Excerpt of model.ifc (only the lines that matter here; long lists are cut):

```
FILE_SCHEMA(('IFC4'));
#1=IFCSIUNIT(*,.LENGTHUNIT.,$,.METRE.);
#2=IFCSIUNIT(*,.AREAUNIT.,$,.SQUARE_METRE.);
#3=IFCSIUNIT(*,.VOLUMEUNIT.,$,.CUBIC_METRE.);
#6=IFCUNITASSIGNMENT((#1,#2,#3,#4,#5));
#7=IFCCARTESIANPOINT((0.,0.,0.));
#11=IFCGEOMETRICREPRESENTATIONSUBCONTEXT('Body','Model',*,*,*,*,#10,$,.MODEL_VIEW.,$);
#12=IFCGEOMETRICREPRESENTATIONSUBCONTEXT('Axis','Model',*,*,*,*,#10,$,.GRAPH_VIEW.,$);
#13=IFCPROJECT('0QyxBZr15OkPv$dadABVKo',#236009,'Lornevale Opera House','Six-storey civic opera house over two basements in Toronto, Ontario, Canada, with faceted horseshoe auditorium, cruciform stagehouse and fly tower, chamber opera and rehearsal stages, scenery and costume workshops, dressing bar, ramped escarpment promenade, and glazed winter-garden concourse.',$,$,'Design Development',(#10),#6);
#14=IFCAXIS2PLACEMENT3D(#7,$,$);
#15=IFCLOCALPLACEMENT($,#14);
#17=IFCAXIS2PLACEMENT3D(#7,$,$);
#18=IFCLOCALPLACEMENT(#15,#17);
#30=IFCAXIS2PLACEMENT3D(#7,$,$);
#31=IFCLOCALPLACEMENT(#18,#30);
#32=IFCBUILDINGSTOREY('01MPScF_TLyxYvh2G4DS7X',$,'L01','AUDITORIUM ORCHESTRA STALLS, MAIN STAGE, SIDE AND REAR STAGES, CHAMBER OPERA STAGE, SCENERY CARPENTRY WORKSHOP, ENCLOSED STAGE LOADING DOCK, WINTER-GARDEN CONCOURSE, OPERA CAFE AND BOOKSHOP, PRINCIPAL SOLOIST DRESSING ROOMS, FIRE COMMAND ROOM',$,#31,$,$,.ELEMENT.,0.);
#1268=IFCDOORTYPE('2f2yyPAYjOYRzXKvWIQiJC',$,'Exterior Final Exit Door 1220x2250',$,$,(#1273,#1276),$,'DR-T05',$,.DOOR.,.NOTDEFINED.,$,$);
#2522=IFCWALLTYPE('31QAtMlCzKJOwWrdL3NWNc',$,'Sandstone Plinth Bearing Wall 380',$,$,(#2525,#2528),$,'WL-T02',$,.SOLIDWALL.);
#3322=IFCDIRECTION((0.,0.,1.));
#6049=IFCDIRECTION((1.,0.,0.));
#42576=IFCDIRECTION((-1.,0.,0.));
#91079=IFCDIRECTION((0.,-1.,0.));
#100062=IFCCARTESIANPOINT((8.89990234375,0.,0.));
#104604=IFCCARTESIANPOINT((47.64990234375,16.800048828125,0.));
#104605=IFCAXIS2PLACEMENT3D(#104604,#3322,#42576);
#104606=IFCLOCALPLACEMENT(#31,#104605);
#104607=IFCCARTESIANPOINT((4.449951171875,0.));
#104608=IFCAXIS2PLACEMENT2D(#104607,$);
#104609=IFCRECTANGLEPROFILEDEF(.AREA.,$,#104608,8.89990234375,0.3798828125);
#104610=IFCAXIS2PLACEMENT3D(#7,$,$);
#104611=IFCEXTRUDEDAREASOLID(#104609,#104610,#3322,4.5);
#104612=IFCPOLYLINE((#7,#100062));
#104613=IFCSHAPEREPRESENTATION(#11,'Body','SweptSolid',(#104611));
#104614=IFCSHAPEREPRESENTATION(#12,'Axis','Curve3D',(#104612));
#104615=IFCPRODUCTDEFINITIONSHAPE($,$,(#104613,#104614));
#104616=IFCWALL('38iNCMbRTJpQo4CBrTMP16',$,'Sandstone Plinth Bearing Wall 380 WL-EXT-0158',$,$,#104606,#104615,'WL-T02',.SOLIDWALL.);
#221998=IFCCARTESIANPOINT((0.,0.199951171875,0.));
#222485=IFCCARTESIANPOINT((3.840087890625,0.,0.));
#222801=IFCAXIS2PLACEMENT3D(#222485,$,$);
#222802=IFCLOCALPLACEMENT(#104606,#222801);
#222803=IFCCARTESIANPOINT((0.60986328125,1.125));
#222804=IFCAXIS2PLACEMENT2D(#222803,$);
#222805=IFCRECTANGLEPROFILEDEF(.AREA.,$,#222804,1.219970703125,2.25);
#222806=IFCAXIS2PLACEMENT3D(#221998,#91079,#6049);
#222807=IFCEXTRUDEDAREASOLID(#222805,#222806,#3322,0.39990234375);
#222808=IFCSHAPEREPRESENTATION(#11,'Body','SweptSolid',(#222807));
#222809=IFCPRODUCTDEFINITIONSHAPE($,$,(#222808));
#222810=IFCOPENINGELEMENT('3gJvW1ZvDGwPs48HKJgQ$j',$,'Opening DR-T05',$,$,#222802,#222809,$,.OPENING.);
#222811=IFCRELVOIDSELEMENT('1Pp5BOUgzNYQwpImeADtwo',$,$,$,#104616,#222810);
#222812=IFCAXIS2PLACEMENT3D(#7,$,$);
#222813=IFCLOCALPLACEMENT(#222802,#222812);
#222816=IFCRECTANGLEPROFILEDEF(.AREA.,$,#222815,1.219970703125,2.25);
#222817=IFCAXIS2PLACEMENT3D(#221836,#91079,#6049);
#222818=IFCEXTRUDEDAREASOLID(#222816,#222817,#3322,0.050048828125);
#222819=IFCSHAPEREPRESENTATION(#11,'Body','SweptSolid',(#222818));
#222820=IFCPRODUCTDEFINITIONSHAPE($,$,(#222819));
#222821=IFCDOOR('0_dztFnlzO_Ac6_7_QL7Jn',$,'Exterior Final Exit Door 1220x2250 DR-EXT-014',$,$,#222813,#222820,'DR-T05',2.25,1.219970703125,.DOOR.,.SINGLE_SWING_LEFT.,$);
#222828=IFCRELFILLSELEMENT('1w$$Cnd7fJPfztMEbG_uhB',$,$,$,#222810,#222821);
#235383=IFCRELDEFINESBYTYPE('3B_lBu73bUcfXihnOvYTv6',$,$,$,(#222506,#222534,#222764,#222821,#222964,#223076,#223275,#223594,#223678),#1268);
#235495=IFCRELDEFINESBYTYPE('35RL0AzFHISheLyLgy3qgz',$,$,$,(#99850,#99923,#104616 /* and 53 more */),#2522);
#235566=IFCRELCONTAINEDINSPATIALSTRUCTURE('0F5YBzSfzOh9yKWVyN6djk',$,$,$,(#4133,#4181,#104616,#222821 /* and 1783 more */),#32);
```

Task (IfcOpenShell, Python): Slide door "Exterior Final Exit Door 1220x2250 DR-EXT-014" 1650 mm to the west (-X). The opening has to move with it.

```python
import ifcopenshell
import ifcopenshell.api.geometry
import ifcopenshell.util.placement
import ifcopenshell.util.unit

model = ifcopenshell.open("model.ifc")
unit_scale = ifcopenshell.util.unit.calculate_unit_scale(model)

door = model.by_id(222821)
opening = door.FillsVoids[0].RelatingOpeningElement
wall = opening.VoidsElements[0].RelatingBuildingElement

wall_matrix = ifcopenshell.util.placement.get_local_placement(wall.ObjectPlacement)
shift = wall_matrix[:3, 0] * 1.65 / unit_scale
before = ifcopenshell.util.placement.get_local_placement(door.ObjectPlacement)[:3, 3].copy()

# The door is placed relative to its opening, so it follows when the opening moves.
matrix = ifcopenshell.util.placement.get_local_placement(opening.ObjectPlacement)
matrix[:3, 3] += shift
ifcopenshell.api.geometry.edit_object_placement(
    model, product=opening, matrix=matrix, is_si=False, should_transform_children=True
)

after = ifcopenshell.util.placement.get_local_placement(door.ObjectPlacement)[:3, 3]
print("door moved by", (after - before).round(3) + 0.0)

model.write("model_rev.ifc")
```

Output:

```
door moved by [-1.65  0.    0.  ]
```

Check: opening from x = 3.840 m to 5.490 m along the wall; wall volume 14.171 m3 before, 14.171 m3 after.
